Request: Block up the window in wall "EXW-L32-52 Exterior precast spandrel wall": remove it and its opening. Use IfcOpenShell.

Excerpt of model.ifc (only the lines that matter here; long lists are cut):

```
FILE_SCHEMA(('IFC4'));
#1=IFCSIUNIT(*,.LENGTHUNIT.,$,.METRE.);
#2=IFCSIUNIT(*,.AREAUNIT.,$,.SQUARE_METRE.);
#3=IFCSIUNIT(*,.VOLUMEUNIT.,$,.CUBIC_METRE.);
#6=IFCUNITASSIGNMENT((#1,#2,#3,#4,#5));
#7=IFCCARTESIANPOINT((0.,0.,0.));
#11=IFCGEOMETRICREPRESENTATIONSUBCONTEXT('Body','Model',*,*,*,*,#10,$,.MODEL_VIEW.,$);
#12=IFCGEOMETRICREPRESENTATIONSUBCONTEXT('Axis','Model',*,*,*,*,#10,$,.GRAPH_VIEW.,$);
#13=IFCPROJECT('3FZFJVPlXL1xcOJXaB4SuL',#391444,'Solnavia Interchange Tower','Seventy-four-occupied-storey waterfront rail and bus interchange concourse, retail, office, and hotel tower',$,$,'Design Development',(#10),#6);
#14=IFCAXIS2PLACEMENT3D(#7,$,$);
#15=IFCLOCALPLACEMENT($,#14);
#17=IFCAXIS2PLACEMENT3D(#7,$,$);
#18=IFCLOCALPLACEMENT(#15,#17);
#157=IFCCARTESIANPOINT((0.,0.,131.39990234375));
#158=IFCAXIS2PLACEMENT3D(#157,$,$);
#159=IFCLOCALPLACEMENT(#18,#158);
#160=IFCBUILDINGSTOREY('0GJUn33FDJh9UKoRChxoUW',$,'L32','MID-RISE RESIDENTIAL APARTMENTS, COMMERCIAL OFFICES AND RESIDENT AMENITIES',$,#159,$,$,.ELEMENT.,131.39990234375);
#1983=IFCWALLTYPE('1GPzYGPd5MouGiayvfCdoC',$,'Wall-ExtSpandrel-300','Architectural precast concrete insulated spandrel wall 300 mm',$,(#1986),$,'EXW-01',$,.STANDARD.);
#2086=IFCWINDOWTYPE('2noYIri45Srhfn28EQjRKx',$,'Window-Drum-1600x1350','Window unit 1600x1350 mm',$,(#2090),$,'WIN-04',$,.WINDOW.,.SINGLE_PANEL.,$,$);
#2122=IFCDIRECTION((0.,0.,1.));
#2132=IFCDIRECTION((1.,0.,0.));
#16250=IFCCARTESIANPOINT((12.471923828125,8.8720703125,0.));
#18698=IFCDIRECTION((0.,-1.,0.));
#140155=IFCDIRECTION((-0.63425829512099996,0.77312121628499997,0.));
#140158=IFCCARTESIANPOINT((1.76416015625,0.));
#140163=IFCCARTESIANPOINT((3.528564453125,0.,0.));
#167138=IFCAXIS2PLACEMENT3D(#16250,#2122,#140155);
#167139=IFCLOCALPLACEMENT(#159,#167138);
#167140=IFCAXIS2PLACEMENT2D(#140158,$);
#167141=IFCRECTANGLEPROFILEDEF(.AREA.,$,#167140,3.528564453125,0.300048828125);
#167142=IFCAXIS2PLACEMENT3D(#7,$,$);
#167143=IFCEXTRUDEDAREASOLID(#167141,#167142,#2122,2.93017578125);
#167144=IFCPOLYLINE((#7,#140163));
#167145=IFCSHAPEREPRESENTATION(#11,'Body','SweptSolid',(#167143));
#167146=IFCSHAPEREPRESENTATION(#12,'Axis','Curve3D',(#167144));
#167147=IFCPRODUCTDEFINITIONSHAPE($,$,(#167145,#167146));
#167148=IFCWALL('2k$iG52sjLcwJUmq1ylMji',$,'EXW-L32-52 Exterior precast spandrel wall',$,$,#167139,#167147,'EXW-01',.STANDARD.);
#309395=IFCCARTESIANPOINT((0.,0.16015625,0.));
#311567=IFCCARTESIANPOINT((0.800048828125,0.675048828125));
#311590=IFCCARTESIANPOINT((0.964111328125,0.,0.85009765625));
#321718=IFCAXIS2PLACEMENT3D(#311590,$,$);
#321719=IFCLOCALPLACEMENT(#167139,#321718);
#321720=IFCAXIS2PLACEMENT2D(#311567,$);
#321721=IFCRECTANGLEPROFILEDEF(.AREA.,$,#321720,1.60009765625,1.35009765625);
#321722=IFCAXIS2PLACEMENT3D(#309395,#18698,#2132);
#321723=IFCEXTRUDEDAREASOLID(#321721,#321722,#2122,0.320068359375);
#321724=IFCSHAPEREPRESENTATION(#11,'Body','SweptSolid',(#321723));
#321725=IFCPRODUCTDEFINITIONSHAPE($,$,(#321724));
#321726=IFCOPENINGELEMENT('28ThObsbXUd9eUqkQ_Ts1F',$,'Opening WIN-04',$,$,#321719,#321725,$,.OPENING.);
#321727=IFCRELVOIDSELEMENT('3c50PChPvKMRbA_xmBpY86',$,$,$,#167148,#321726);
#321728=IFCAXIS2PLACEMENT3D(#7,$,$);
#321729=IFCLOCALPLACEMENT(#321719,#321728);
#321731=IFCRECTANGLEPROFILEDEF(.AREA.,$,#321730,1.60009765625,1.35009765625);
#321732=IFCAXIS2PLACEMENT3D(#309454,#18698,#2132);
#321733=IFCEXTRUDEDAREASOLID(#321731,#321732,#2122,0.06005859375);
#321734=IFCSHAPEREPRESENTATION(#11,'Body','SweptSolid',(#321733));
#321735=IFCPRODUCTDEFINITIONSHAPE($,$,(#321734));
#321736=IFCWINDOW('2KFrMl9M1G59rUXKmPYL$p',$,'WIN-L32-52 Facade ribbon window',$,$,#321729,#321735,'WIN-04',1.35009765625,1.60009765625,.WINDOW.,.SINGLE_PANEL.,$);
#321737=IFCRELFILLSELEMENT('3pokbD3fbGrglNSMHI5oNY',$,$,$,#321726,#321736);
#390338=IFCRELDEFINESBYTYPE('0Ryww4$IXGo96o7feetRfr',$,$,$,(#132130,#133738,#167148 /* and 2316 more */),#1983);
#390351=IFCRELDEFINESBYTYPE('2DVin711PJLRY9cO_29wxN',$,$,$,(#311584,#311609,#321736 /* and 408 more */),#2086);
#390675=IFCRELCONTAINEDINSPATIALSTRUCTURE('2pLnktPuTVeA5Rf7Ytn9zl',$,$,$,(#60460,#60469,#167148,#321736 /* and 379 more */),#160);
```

```python
import ifcopenshell
import ifcopenshell.api.feature
import ifcopenshell.api.root
import ifcopenshell.geom
import ifcopenshell.util.shape

model = ifcopenshell.open("model.ifc")
settings = ifcopenshell.geom.settings()


def volume(element):
    """Net volume in cubic metres, openings subtracted."""
    shape = ifcopenshell.geom.create_shape(settings, element)
    return ifcopenshell.util.shape.get_volume(shape.geometry)


window = model.by_guid("2KFrMl9M1G59rUXKmPYL$p")
opening = window.FillsVoids[0].RelatingOpeningElement
wall = opening.VoidsElements[0].RelatingBuildingElement
before = volume(wall)

ifcopenshell.api.root.remove_product(model, product=window)
ifcopenshell.api.feature.remove_feature(model, feature=opening)

after = volume(wall)

print(f"wall volume {before:.3f} -> {after:.3f} m3")

model.write("model_edited.ifc")
```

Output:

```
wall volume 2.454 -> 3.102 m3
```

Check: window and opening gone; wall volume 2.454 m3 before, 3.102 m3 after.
